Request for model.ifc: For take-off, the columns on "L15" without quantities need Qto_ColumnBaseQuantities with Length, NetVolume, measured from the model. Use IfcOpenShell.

First a look at what the model holds.

```python
import ifcopenshell
import ifcopenshell.util.element
import ifcopenshell.util.unit

model = ifcopenshell.open("model.ifc")
print(model.schema)
for unit_type in ("LENGTHUNIT", "AREAUNIT", "VOLUMEUNIT"):
    print(unit_type, ifcopenshell.util.unit.calculate_unit_scale(model, unit_type))
storey = next(s for s in model.by_type("IfcBuildingStorey") if s.Name == "L15")
columns = [e for e in ifcopenshell.util.element.get_decomposition(storey) if e.is_a("IfcColumn")]
for e in sorted(columns, key=lambda e: e.id()):
    print(e.id(), e.is_a(), e.Name, list(ifcopenshell.util.element.get_psets(e, qtos_only=True)), sep=" | ")
```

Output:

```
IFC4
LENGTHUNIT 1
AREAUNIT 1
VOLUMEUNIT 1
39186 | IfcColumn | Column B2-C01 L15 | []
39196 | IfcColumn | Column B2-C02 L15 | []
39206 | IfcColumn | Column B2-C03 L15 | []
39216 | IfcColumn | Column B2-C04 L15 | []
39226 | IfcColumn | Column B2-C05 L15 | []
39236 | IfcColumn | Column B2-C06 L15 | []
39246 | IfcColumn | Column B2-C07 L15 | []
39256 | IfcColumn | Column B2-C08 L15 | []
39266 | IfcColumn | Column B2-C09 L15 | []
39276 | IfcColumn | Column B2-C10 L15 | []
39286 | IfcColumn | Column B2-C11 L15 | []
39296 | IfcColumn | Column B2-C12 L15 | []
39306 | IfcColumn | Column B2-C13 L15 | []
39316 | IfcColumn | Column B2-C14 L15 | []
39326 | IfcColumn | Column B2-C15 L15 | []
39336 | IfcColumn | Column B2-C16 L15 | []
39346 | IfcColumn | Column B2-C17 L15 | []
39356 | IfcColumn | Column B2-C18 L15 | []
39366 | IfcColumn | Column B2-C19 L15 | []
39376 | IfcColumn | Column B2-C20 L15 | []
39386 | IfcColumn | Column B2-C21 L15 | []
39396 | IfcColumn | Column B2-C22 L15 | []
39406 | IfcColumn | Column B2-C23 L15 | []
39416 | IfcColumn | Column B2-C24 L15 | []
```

```python
import ifcopenshell
import ifcopenshell.api.pset
import ifcopenshell.geom
import ifcopenshell.util.element
import ifcopenshell.util.shape
import ifcopenshell.util.unit

model = ifcopenshell.open("model.ifc")
unit_scale = ifcopenshell.util.unit.calculate_unit_scale(model)
volume_scale = ifcopenshell.util.unit.calculate_unit_scale(model, "VOLUMEUNIT")
settings = ifcopenshell.geom.settings()

storey = next(s for s in model.by_type("IfcBuildingStorey") if s.Name == "L15")
columns = [e for e in ifcopenshell.util.element.get_decomposition(storey) if e.is_a("IfcColumn")]

for e in sorted(columns, key=lambda e: e.id()):
    if ifcopenshell.util.element.get_psets(e, qtos_only=True, should_inherit=False):
        continue
    # Geometry comes back in metres, in the element's own axes.
    shape = ifcopenshell.geom.create_shape(settings, e)
    values = {
        "Length": ifcopenshell.util.shape.get_z(shape.geometry) / unit_scale,
        "NetVolume": ifcopenshell.util.shape.get_volume(shape.geometry) / volume_scale,
    }
    qto = ifcopenshell.api.pset.add_qto(model, product=e, name="Qto_ColumnBaseQuantities")
    ifcopenshell.api.pset.edit_qto(model, qto=qto, properties=values)
    print(e.id(), {k: round(v, 3) for k, v in values.items()})

model.write("model_rev.ifc")
```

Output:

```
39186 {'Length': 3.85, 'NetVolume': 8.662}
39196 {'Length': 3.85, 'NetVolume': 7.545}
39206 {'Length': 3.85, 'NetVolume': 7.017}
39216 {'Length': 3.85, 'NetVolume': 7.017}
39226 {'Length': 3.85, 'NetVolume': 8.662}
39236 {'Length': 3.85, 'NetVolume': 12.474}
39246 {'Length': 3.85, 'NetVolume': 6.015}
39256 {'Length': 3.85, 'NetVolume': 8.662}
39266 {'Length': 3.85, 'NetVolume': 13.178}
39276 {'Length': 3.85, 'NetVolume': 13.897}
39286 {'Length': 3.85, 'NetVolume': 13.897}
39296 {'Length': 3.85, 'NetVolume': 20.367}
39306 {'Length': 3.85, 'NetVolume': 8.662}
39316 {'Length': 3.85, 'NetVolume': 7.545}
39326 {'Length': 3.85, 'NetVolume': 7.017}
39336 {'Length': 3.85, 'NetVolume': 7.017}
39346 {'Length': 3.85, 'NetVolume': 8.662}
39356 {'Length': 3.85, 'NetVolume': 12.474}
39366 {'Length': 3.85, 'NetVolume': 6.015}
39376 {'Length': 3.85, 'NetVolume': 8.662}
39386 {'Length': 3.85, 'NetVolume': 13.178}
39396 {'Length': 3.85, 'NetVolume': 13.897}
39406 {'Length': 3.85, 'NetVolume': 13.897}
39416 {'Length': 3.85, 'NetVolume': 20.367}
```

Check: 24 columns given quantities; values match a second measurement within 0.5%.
